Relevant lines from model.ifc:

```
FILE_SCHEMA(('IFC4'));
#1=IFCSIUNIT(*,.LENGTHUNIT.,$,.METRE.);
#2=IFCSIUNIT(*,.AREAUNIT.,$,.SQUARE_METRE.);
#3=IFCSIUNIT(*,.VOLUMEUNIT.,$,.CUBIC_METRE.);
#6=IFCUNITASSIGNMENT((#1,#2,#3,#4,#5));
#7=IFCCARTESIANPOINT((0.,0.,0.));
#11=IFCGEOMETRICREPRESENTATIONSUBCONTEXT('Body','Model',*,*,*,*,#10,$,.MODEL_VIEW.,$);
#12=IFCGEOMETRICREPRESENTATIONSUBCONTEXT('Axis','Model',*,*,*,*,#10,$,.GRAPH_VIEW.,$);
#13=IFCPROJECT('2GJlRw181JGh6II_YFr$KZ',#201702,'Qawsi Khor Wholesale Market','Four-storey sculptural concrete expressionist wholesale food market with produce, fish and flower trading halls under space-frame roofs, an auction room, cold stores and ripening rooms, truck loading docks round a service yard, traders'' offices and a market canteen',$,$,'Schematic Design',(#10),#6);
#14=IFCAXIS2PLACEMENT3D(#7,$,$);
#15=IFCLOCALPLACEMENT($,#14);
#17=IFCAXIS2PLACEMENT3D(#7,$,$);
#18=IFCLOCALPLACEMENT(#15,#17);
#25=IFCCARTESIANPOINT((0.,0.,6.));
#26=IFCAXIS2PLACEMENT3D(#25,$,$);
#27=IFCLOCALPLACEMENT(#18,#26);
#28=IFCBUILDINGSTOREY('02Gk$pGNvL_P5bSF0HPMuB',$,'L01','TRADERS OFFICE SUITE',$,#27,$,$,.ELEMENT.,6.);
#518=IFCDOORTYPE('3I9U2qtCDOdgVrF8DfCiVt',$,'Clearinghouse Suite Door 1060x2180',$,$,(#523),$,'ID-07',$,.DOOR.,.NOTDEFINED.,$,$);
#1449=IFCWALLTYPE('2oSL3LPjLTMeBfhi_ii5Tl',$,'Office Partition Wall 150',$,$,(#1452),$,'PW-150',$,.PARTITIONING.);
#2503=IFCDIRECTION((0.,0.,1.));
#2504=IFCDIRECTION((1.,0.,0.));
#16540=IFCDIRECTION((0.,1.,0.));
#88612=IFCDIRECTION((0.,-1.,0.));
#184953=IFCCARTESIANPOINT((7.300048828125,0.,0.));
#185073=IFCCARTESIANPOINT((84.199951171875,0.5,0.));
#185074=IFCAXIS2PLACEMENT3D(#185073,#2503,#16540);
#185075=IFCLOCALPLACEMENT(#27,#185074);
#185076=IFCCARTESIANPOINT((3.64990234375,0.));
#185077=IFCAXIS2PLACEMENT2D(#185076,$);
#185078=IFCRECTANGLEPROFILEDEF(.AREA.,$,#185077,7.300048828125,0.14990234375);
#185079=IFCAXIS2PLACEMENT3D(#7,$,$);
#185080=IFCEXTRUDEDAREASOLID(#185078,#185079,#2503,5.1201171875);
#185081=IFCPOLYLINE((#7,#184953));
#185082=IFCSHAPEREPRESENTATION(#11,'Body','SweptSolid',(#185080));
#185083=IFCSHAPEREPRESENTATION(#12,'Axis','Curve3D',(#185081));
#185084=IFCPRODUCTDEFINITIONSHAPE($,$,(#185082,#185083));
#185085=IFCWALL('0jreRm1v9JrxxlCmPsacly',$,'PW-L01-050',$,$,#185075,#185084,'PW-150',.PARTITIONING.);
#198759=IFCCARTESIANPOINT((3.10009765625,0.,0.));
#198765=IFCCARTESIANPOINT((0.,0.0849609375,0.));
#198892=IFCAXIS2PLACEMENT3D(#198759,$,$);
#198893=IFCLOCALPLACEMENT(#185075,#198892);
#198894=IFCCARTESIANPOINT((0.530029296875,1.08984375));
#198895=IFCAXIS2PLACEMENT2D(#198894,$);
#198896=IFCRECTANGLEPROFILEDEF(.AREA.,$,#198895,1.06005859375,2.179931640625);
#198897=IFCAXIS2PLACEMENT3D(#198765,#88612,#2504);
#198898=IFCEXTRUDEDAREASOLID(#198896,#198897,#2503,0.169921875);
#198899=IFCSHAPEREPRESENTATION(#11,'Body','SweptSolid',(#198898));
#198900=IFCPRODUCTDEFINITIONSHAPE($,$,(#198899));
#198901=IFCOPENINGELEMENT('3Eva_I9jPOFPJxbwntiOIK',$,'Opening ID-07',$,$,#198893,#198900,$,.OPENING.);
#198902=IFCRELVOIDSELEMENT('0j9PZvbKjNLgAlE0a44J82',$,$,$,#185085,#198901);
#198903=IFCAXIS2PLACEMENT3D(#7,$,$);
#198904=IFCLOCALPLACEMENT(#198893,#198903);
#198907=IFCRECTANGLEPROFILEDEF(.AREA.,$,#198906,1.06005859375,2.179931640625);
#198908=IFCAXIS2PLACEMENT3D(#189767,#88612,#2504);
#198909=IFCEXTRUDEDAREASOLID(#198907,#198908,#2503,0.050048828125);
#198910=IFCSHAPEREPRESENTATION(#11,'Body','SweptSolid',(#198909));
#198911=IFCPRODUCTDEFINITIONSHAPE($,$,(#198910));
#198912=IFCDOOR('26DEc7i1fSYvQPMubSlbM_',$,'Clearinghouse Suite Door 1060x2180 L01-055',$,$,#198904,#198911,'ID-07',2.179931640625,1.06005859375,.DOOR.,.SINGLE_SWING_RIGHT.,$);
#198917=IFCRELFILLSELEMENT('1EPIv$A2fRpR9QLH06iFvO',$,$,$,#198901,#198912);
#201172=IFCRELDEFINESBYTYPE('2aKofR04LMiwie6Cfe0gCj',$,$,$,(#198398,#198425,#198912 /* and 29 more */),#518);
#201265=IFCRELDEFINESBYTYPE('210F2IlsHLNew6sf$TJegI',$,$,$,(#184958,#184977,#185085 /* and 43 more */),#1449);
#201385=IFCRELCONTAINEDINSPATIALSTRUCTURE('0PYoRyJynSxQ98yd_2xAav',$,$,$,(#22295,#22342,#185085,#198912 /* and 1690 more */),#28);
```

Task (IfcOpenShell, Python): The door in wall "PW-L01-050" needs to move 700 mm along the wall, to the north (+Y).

```python
import ifcopenshell
import ifcopenshell.api.geometry
import ifcopenshell.util.placement

model = ifcopenshell.open("model.ifc")

door = model.by_id(198912)
opening = door.FillsVoids[0].RelatingOpeningElement
wall = opening.VoidsElements[0].RelatingBuildingElement

wall_matrix = ifcopenshell.util.placement.get_local_placement(wall.ObjectPlacement)
shift = wall_matrix[:3, 0] * 0.7
before = ifcopenshell.util.placement.get_local_placement(door.ObjectPlacement)[:3, 3].copy()

# The door is placed relative to its opening, so it follows when the opening moves.
matrix = ifcopenshell.util.placement.get_local_placement(opening.ObjectPlacement)
matrix[:3, 3] += shift
ifcopenshell.api.geometry.edit_object_placement(
    model, product=opening, matrix=matrix, is_si=False, should_transform_children=True
)

after = ifcopenshell.util.placement.get_local_placement(door.ObjectPlacement)[:3, 3]
print("door moved by", (after - before).round(3) + 0.0)

model.write("model_edited.ifc")
```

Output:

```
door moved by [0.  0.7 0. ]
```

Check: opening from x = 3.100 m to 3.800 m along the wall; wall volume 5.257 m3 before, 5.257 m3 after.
